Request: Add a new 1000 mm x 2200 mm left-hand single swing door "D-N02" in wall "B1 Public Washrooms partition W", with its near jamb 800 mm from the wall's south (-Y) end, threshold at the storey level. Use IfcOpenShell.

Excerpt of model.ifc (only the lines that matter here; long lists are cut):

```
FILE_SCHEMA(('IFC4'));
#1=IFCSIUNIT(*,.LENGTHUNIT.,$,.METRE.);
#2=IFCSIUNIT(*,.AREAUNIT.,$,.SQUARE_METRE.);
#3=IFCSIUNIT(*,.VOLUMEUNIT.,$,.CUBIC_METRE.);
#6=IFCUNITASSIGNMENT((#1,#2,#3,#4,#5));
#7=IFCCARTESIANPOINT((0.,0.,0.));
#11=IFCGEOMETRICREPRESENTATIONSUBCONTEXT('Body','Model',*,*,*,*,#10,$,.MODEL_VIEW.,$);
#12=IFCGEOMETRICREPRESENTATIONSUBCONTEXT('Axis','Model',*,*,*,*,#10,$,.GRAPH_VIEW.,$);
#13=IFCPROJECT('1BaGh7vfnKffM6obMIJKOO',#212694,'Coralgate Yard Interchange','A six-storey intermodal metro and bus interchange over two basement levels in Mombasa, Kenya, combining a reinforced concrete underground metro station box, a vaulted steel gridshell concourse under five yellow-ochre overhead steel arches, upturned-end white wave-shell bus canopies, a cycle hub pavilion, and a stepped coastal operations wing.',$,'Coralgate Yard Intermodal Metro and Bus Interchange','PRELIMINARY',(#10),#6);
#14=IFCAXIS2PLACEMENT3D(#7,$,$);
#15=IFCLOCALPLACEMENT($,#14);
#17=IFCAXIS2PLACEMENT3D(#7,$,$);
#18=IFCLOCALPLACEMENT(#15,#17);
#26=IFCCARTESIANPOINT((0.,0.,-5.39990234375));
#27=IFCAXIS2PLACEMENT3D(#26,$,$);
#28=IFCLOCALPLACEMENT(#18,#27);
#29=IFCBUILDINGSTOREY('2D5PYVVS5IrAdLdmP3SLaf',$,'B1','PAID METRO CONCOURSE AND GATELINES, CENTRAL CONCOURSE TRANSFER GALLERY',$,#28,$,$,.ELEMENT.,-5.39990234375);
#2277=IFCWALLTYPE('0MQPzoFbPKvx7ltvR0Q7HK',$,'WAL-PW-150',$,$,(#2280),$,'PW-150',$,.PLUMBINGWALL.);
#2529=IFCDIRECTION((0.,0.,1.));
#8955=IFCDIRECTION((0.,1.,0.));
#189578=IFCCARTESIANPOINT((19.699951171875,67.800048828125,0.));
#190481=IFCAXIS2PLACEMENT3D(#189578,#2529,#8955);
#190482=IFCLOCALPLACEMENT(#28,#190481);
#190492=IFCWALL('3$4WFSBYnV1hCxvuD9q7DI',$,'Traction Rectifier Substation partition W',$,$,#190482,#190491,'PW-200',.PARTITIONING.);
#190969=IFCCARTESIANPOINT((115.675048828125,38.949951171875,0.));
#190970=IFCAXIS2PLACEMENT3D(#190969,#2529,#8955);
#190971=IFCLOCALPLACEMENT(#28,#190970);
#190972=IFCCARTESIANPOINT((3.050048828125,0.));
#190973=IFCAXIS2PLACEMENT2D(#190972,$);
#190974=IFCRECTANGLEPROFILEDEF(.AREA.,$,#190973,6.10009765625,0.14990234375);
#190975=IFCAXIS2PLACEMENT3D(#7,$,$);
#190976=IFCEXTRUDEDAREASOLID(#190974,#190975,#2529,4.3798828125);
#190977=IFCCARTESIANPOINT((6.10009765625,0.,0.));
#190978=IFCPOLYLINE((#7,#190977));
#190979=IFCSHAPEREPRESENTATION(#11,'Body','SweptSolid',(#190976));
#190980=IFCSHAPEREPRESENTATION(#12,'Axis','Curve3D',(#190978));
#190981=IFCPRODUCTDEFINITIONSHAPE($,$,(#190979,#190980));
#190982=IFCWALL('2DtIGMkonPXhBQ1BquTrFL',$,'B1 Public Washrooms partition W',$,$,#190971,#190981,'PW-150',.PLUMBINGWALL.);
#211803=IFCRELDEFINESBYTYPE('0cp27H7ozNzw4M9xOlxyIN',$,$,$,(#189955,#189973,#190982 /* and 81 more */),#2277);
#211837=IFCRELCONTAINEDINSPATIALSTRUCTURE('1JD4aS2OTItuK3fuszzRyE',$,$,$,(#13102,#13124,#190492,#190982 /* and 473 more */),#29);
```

```python
import numpy as np
import ifcopenshell
import ifcopenshell.api.feature
import ifcopenshell.api.geometry
import ifcopenshell.api.root
import ifcopenshell.api.spatial
import ifcopenshell.geom
import ifcopenshell.util.element
import ifcopenshell.util.placement
import ifcopenshell.util.representation
import ifcopenshell.util.shape
import ifcopenshell.util.unit

model = ifcopenshell.open("model.ifc")
unit_scale = ifcopenshell.util.unit.calculate_unit_scale(model)
settings = ifcopenshell.geom.settings()


def volume(element):
    """Net volume in cubic metres, openings subtracted."""
    shape = ifcopenshell.geom.create_shape(settings, element)
    return ifcopenshell.util.shape.get_volume(shape.geometry)


wall = model.by_guid("2DtIGMkonPXhBQ1BquTrFL")
storey = ifcopenshell.util.element.get_container(wall, ifc_class="IfcBuildingStorey")
context = ifcopenshell.util.representation.get_context(model, "Model", "Body", "MODEL_VIEW")
before = volume(wall)

width, height, from_end, sill = 1, 2.2, 0.8, 0.0  # metres

# The wall runs along its own X axis, and the end named is its -X end.
wall_shape = ifcopenshell.geom.create_shape(settings, wall)
x, y, z = ifcopenshell.util.shape.get_vertices(wall_shape.geometry).T
start = x.min() + from_end
face, thickness = float(y.min()), float(y.max() - y.min())
wall_matrix = ifcopenshell.util.placement.get_local_placement(wall.ObjectPlacement)
level = ifcopenshell.util.placement.get_local_placement(storey.ObjectPlacement)[2, 3]


def in_wall(x, y):
    """Placement at x, y metres in the wall's axes, at sill height."""
    matrix = wall_matrix.copy()
    matrix[:, 3] = wall_matrix @ np.array([x / unit_scale, y / unit_scale, 0.0, 1.0])
    matrix[2, 3] = level + sill / unit_scale
    return matrix


# Opening: a box that overshoots both wall faces by 50 mm.
opening = ifcopenshell.api.root.create_entity(model, ifc_class="IfcOpeningElement", predefined_type="OPENING")
box = ifcopenshell.api.geometry.add_wall_representation(
    model, context=context, length=width, height=height, thickness=thickness + 0.1
)
ifcopenshell.api.geometry.assign_representation(model, product=opening, representation=box)
ifcopenshell.api.geometry.edit_object_placement(model, product=opening, matrix=in_wall(start, face - 0.05), is_si=False)
ifcopenshell.api.feature.add_feature(model, feature=opening, element=wall)

door = ifcopenshell.api.root.create_entity(model, ifc_class="IfcDoor", name="D-N02", predefined_type="DOOR")
door.OverallWidth, door.OverallHeight = width / unit_scale, height / unit_scale
door.OperationType = "SINGLE_SWING_LEFT"
body = ifcopenshell.api.geometry.add_door_representation(
    model,
    context=context,
    overall_width=door.OverallWidth,
    overall_height=door.OverallHeight,
    operation_type="SINGLE_SWING_LEFT",
    lining_properties={"LiningDepth": thickness / unit_scale, "ThresholdDepth": thickness / unit_scale},
)
ifcopenshell.api.geometry.assign_representation(model, product=door, representation=body)
ifcopenshell.api.spatial.assign_container(model, products=[door], relating_structure=storey)
ifcopenshell.api.feature.add_filling(model, opening=opening, element=door)

# The lining spans the wall, so the door starts at the wall face.
ifcopenshell.api.geometry.edit_object_placement(model, product=door, matrix=in_wall(start, face), is_si=False)

after = volume(wall)

print(f"wall volume {before:.3f} -> {after:.3f} m3")

model.write("model-out.ifc")
```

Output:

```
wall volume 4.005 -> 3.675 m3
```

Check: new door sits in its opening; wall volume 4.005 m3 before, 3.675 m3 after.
